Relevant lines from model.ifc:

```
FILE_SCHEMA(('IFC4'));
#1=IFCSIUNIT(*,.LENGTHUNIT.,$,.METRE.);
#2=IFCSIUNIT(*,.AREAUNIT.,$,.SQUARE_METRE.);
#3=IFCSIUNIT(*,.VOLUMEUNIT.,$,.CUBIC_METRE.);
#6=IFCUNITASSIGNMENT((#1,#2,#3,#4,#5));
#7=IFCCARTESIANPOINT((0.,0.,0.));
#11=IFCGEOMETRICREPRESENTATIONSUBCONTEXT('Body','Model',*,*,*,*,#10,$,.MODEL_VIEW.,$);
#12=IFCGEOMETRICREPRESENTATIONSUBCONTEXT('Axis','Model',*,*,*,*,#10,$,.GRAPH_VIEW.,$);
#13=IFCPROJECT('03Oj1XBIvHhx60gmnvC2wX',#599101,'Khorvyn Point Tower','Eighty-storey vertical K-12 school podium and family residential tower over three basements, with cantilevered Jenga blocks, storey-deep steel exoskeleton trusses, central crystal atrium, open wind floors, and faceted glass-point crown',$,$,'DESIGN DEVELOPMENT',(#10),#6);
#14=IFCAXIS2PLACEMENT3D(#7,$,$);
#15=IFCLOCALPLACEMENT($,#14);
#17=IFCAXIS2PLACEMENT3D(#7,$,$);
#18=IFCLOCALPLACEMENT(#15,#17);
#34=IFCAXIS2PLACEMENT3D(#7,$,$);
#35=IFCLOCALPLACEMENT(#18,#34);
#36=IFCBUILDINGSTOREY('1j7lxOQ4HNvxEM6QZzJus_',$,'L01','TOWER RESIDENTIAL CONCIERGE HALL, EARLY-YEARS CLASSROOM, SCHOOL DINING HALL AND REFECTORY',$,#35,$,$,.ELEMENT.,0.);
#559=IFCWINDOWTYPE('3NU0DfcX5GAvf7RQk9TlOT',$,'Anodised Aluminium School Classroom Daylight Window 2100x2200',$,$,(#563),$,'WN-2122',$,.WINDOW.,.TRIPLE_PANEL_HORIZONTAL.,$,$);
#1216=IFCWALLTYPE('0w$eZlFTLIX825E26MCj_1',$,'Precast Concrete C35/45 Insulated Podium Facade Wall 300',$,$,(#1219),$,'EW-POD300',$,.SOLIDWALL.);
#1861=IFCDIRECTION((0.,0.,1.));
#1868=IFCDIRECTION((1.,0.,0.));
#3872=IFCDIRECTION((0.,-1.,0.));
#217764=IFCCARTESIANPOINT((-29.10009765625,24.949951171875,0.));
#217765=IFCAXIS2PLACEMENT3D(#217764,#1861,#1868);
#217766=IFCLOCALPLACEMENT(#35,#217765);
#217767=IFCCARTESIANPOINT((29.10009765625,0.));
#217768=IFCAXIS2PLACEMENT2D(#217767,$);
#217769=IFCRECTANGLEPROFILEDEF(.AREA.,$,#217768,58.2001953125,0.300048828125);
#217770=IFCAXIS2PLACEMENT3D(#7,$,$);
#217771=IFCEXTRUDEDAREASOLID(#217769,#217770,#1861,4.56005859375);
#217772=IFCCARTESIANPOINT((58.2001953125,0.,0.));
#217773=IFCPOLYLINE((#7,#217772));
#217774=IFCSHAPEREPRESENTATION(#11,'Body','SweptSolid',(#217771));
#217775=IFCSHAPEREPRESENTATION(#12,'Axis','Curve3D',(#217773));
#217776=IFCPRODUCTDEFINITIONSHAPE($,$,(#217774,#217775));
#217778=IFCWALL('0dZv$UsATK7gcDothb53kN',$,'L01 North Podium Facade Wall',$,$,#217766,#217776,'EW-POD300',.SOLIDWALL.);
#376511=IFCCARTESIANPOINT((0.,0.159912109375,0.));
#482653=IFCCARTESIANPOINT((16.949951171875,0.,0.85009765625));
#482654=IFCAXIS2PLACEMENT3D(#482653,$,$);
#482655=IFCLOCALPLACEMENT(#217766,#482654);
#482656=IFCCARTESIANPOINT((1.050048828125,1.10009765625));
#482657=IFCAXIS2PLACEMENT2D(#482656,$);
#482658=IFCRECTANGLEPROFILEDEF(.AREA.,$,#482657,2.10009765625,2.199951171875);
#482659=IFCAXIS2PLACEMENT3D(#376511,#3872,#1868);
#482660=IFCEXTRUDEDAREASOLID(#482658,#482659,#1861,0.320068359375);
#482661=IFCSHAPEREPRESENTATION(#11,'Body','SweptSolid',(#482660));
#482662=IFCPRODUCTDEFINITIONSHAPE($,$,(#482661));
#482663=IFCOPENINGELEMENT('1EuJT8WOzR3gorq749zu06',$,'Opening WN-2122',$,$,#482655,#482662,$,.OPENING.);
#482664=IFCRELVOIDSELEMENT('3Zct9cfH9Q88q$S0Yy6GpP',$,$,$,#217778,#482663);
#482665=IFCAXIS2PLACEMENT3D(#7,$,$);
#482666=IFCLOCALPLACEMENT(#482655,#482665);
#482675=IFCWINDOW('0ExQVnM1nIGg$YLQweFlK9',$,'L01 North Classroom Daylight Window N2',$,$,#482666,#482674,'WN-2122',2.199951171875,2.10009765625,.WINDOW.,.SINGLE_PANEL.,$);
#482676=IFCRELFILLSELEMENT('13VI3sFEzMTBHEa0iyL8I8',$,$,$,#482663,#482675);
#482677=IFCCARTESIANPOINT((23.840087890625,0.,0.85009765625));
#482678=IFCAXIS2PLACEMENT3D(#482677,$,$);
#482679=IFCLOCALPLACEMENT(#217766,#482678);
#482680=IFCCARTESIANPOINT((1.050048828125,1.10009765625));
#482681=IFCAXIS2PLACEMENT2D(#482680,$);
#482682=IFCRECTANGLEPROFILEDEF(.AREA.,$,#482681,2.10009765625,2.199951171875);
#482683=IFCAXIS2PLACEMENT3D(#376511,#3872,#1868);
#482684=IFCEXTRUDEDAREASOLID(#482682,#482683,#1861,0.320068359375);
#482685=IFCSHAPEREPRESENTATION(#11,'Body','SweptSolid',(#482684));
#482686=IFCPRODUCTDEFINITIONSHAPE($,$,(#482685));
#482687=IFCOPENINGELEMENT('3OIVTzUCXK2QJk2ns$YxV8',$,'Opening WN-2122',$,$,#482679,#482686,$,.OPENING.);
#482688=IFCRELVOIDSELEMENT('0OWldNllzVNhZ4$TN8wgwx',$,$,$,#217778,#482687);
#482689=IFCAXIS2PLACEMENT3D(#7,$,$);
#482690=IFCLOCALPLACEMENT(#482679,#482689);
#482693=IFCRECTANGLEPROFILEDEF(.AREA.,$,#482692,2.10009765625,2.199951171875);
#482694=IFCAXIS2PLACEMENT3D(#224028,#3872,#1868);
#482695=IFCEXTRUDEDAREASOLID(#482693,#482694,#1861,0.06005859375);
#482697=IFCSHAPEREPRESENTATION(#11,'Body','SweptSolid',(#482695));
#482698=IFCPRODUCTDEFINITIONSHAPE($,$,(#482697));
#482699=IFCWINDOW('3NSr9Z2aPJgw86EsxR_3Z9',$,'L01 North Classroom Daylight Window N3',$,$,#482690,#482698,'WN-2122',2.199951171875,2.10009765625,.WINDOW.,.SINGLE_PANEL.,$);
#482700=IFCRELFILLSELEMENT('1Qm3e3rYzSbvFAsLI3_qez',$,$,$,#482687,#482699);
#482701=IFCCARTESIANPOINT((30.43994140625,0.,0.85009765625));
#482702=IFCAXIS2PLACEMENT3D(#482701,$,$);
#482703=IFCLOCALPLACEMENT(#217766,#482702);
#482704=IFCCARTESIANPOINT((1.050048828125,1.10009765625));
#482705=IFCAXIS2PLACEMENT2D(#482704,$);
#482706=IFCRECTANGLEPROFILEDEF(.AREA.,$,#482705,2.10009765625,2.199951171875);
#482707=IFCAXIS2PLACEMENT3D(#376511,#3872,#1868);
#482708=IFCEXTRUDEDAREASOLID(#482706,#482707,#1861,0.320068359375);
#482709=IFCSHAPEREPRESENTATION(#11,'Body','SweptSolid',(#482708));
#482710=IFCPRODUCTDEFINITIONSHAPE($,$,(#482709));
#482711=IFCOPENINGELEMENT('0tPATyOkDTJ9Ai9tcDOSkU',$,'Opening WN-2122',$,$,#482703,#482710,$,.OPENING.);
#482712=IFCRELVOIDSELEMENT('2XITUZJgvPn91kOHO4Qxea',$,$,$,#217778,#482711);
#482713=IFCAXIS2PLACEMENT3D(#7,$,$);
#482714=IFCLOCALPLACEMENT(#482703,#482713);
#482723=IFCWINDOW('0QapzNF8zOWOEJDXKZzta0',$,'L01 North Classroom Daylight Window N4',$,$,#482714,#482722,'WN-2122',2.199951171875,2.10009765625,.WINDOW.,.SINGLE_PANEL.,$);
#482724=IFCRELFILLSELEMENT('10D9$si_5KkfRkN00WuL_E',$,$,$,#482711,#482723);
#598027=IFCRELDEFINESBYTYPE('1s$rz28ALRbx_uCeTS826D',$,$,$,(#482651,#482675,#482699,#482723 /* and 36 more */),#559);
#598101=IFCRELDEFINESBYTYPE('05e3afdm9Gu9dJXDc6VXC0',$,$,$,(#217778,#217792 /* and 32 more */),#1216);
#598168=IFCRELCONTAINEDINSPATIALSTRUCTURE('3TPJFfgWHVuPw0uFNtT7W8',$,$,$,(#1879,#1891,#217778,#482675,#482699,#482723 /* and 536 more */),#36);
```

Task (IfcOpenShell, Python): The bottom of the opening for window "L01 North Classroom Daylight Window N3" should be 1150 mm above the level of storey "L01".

```python
import numpy as np
import ifcopenshell
import ifcopenshell.api.geometry
import ifcopenshell.geom
import ifcopenshell.util.element
import ifcopenshell.util.placement
import ifcopenshell.util.shape
import ifcopenshell.util.unit

model = ifcopenshell.open("model.ifc")
unit_scale = ifcopenshell.util.unit.calculate_unit_scale(model)

window = model.by_id(482699)
opening = window.FillsVoids[0].RelatingOpeningElement
storey = ifcopenshell.util.element.get_container(window, ifc_class="IfcBuildingStorey")
level = ifcopenshell.util.placement.get_local_placement(storey.ObjectPlacement)[2, 3]

# The opening's origin need not be at the sill, so measure its lowest point.
shape = ifcopenshell.geom.create_shape(ifcopenshell.geom.settings(), opening)
bottom = ifcopenshell.util.shape.get_shape_bottom_elevation(shape, shape.geometry) / unit_scale
dz = level + 1.15 / unit_scale - bottom

shift = np.array([0.0, 0.0, dz])
# The window is placed relative to its opening, so it follows when the opening moves.
matrix = ifcopenshell.util.placement.get_local_placement(opening.ObjectPlacement)
matrix[:3, 3] += shift
ifcopenshell.api.geometry.edit_object_placement(
    model, product=opening, matrix=matrix, is_si=False, should_transform_children=True
)

print(f"moved by {dz * unit_scale:+.3f} m")

model.write("model-out.ifc")
```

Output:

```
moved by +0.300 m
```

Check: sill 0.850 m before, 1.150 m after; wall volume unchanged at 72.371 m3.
